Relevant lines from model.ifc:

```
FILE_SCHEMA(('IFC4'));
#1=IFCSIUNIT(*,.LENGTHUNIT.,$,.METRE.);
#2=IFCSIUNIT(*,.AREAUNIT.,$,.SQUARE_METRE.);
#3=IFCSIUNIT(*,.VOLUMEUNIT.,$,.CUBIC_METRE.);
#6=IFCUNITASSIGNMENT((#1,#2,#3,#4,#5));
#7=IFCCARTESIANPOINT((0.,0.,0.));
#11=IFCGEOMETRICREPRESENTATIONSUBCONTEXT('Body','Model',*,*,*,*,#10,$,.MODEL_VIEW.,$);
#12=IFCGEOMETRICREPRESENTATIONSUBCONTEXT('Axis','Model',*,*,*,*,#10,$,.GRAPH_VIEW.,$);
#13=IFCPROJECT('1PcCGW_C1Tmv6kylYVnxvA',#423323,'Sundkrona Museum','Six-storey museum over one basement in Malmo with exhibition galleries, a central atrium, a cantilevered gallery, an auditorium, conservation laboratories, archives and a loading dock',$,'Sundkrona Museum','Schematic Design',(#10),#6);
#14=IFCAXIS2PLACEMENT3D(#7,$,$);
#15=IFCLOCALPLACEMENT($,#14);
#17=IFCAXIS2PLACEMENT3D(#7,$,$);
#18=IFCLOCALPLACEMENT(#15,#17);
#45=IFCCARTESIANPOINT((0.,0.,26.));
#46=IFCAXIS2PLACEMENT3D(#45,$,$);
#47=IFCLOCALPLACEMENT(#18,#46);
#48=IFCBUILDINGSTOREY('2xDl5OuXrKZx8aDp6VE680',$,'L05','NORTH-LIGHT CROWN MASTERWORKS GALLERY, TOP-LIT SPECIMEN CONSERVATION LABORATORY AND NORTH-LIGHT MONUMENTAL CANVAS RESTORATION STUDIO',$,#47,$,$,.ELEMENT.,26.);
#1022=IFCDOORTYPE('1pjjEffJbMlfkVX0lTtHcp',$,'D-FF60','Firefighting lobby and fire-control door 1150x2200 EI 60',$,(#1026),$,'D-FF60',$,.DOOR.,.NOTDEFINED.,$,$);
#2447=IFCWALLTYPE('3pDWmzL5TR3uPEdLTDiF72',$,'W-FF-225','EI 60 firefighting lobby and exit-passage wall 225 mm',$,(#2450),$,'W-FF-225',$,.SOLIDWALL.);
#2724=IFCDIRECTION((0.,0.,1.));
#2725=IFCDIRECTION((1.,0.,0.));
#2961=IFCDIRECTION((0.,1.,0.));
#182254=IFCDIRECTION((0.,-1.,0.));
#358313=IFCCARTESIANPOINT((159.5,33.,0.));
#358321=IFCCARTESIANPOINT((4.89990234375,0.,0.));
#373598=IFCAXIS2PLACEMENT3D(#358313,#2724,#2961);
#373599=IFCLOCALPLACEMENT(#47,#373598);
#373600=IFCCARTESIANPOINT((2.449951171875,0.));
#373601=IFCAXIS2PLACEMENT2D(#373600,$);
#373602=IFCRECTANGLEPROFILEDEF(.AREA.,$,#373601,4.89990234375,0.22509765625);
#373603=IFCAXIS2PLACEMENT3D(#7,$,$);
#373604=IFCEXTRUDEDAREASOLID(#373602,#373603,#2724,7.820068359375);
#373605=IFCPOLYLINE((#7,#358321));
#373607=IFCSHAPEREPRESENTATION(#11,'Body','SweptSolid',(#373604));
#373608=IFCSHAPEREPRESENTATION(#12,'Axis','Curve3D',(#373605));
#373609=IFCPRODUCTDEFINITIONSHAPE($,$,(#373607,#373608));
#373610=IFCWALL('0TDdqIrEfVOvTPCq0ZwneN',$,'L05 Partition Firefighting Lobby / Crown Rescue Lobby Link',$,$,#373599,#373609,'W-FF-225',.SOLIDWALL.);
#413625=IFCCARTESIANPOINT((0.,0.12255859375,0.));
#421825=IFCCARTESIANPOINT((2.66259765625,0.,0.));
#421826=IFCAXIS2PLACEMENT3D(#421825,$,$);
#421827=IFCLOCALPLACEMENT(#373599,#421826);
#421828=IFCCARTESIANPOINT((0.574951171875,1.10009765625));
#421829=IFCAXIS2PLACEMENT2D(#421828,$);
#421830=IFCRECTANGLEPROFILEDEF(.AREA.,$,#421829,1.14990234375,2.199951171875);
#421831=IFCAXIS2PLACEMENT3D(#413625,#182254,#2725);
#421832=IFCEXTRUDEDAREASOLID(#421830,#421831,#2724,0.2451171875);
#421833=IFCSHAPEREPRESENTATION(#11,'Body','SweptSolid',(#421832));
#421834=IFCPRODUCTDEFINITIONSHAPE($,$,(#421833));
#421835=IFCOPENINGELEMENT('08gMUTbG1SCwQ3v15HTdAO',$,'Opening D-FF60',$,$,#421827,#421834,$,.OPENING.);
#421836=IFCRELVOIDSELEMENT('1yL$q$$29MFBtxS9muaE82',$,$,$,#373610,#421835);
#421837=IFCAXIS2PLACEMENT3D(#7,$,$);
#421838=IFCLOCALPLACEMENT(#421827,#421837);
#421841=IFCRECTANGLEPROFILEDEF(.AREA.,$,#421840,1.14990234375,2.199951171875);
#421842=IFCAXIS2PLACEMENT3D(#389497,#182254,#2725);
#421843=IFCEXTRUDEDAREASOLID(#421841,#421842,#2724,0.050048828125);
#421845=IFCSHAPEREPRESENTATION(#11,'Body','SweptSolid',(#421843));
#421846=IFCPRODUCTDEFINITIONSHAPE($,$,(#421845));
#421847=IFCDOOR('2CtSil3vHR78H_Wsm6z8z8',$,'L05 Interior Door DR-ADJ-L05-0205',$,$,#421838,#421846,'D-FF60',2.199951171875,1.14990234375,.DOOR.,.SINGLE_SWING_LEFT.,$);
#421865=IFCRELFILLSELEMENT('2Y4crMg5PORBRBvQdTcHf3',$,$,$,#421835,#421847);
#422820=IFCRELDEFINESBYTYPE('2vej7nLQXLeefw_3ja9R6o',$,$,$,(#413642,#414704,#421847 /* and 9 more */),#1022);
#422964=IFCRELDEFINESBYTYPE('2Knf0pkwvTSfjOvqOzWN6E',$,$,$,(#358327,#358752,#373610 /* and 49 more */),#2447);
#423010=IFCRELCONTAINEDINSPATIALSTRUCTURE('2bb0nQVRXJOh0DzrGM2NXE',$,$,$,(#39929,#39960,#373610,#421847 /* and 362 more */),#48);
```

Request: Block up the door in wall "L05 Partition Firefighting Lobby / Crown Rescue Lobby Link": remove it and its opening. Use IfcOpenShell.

```python
import ifcopenshell
import ifcopenshell.api.feature
import ifcopenshell.api.root
import ifcopenshell.geom
import ifcopenshell.util.shape

model = ifcopenshell.open("model.ifc")
settings = ifcopenshell.geom.settings()


def volume(element):
    """Net volume in cubic metres, openings subtracted."""
    shape = ifcopenshell.geom.create_shape(settings, element)
    return ifcopenshell.util.shape.get_volume(shape.geometry)


door = model.by_guid("2CtSil3vHR78H_Wsm6z8z8")
opening = door.FillsVoids[0].RelatingOpeningElement
wall = opening.VoidsElements[0].RelatingBuildingElement
before = volume(wall)

ifcopenshell.api.root.remove_product(model, product=door)
ifcopenshell.api.feature.remove_feature(model, feature=opening)

after = volume(wall)

print(f"wall volume {before:.3f} -> {after:.3f} m3")

model.write("model-out.ifc")
```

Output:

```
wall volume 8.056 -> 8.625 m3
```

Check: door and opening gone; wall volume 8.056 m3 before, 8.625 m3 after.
